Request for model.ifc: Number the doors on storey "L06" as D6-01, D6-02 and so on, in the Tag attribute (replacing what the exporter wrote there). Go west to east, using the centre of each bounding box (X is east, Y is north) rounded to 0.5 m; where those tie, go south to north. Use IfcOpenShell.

First a look at what the model holds.

```python
import ifcopenshell
import ifcopenshell.util.element
import ifcopenshell.util.placement

model = ifcopenshell.open("model.ifc")
print(model.schema)
storey = next(s for s in model.by_type("IfcBuildingStorey") if s.Name == "L06")
doors = [e for e in ifcopenshell.util.element.get_decomposition(storey) if e.is_a("IfcDoor")]
for e in sorted(doors, key=lambda e: e.id()):
    origin = ifcopenshell.util.placement.get_local_placement(e.ObjectPlacement)[:3, 3]
    print(e.id(), e.Tag, e.Name, origin.round(2) + 0.0, sep=" | ")
```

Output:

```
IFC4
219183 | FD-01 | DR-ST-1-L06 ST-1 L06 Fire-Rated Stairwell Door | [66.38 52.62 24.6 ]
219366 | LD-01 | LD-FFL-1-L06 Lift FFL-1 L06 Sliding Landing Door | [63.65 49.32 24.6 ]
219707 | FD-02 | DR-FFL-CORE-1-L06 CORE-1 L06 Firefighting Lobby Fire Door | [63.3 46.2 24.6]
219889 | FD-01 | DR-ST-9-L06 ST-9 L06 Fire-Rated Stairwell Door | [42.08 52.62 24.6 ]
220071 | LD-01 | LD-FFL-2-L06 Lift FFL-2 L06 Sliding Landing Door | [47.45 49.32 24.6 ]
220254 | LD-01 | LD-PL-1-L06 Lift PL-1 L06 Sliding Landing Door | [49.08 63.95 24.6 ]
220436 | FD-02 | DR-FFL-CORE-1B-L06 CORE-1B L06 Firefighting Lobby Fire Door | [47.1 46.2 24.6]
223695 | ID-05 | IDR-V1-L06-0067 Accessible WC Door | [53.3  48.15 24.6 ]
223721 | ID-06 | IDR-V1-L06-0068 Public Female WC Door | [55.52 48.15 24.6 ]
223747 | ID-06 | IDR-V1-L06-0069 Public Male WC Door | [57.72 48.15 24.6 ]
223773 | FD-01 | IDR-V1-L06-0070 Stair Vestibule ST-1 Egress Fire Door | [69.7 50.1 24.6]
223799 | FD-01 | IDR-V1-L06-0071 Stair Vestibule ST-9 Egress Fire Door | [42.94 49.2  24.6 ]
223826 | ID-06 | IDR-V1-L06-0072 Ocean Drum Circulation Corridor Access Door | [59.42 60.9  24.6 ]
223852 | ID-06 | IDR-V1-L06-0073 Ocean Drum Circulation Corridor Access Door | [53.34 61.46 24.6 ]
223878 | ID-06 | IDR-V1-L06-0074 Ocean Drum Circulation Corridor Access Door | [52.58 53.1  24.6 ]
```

```python
import ifcopenshell
import ifcopenshell.geom
import ifcopenshell.util.element
import ifcopenshell.util.shape

model = ifcopenshell.open("model.ifc")
settings = ifcopenshell.geom.settings()
settings.set("use-world-coords", True)


def centre(element):
    shape = ifcopenshell.geom.create_shape(settings, element)
    return ifcopenshell.util.shape.get_bbox_centroid(shape.geometry)


storey = next(s for s in model.by_type("IfcBuildingStorey") if s.Name == "L06")
doors = [e for e in ifcopenshell.util.element.get_decomposition(storey) if e.is_a("IfcDoor")]

# Insertion points can sit at a corner or the storey origin, so sort by the geometry (in metres).
centres = {e: centre(e) for e in doors}
doors.sort(key=lambda e: (round(centres[e][0] / 0.5), centres[e][1]))

for i, e in enumerate(doors, start=1):
    number = f"D6-{i:02d}"
    e.Tag = number
    print(e.id(), number)

model.write("model_rev.ifc")
```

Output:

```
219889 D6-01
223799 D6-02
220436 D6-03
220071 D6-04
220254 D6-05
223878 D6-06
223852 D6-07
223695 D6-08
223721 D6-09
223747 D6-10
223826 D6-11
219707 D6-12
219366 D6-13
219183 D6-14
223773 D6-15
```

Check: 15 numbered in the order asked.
